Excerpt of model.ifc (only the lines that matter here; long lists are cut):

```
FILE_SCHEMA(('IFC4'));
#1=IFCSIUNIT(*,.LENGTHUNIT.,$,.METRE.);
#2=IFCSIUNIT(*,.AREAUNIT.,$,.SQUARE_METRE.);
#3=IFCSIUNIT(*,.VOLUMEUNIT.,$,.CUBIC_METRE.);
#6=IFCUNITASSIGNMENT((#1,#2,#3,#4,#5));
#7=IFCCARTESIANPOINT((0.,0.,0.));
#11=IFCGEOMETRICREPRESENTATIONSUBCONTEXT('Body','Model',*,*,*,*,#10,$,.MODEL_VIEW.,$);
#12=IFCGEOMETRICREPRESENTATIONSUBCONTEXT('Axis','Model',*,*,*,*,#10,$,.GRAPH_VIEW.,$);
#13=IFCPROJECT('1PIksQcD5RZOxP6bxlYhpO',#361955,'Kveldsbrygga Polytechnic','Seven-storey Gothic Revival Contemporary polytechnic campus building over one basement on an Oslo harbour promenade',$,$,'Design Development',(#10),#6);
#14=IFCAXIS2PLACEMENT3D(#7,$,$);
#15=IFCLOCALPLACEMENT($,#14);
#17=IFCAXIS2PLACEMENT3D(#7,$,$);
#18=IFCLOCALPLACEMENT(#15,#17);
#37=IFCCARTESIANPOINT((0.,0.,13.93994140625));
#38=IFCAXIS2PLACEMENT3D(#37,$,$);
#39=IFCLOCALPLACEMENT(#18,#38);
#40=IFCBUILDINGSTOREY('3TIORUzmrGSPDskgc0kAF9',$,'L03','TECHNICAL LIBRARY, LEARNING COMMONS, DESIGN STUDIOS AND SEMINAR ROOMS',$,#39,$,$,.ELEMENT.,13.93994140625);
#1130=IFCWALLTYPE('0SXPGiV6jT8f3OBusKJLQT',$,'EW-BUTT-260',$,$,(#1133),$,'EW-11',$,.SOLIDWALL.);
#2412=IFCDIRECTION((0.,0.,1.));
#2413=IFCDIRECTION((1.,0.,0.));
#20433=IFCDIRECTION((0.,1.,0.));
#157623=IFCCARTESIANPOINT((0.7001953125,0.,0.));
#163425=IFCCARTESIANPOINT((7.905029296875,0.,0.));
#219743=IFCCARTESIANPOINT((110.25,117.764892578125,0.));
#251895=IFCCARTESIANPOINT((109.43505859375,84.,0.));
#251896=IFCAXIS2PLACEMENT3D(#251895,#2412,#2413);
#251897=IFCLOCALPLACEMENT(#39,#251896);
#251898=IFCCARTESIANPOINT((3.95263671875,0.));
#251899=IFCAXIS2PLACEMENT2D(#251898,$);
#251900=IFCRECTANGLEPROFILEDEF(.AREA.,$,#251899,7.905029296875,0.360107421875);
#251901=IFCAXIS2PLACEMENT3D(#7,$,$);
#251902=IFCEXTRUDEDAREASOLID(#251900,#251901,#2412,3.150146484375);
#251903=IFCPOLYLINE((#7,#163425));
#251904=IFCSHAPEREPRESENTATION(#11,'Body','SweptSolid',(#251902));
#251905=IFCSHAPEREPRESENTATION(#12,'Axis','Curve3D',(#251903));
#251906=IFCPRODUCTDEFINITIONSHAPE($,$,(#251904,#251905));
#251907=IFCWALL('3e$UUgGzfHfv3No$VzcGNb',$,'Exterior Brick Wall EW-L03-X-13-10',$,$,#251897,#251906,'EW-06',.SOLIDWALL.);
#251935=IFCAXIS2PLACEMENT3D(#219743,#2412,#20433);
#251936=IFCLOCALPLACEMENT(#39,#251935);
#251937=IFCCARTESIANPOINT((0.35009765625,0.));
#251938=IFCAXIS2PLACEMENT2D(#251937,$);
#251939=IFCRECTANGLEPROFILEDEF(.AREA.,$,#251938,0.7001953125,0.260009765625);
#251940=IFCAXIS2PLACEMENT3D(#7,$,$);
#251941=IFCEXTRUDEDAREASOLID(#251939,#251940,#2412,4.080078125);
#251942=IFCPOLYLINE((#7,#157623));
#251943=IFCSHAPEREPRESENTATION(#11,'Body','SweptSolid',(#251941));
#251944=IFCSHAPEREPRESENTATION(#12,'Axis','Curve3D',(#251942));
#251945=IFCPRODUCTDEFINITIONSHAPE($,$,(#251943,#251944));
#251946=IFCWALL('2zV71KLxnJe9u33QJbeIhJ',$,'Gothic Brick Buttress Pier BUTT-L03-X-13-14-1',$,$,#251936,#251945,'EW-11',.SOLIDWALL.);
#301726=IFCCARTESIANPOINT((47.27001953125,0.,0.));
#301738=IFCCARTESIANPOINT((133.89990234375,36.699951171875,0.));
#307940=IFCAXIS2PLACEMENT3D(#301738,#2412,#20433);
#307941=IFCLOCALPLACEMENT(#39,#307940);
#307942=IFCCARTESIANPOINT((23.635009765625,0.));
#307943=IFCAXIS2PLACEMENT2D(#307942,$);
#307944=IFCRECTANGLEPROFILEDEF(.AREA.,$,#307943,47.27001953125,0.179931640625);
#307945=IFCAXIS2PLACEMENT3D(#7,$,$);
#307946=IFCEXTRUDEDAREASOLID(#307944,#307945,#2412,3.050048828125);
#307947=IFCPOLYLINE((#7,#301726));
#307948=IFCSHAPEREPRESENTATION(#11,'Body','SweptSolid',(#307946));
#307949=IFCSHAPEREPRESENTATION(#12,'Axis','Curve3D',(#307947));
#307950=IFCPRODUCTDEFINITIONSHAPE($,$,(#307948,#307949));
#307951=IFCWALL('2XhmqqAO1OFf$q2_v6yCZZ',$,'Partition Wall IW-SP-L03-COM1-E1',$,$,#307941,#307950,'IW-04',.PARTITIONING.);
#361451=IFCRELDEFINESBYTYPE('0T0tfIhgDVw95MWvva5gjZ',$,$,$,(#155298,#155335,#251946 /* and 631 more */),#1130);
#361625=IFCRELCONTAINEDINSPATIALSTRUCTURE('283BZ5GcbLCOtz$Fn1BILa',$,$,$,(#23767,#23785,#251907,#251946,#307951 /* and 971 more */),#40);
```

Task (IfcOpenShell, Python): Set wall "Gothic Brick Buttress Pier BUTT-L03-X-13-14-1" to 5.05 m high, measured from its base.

```python
import ifcopenshell
import ifcopenshell.geom
import ifcopenshell.util.representation
import ifcopenshell.util.shape

model = ifcopenshell.open("model.ifc")
settings = ifcopenshell.geom.settings()


def volume(element):
    """Net volume in cubic metres, openings subtracted."""
    shape = ifcopenshell.geom.create_shape(settings, element)
    return ifcopenshell.util.shape.get_volume(shape.geometry)


wall = model.by_guid("2zV71KLxnJe9u33QJbeIhJ")
before = volume(wall)

body = ifcopenshell.util.representation.get_representation(wall, "Model", "Body")
solid = body.Items[0]
old_height = solid.Depth
solid.Depth = 5.05
after = volume(wall)

print(f"height {old_height:g} -> {solid.Depth:g}, volume {before:.3f} -> {after:.3f} m3")

model.write("model_edited.ifc")
```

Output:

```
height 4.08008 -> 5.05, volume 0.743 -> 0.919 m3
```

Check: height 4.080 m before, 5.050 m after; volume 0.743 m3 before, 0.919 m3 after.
